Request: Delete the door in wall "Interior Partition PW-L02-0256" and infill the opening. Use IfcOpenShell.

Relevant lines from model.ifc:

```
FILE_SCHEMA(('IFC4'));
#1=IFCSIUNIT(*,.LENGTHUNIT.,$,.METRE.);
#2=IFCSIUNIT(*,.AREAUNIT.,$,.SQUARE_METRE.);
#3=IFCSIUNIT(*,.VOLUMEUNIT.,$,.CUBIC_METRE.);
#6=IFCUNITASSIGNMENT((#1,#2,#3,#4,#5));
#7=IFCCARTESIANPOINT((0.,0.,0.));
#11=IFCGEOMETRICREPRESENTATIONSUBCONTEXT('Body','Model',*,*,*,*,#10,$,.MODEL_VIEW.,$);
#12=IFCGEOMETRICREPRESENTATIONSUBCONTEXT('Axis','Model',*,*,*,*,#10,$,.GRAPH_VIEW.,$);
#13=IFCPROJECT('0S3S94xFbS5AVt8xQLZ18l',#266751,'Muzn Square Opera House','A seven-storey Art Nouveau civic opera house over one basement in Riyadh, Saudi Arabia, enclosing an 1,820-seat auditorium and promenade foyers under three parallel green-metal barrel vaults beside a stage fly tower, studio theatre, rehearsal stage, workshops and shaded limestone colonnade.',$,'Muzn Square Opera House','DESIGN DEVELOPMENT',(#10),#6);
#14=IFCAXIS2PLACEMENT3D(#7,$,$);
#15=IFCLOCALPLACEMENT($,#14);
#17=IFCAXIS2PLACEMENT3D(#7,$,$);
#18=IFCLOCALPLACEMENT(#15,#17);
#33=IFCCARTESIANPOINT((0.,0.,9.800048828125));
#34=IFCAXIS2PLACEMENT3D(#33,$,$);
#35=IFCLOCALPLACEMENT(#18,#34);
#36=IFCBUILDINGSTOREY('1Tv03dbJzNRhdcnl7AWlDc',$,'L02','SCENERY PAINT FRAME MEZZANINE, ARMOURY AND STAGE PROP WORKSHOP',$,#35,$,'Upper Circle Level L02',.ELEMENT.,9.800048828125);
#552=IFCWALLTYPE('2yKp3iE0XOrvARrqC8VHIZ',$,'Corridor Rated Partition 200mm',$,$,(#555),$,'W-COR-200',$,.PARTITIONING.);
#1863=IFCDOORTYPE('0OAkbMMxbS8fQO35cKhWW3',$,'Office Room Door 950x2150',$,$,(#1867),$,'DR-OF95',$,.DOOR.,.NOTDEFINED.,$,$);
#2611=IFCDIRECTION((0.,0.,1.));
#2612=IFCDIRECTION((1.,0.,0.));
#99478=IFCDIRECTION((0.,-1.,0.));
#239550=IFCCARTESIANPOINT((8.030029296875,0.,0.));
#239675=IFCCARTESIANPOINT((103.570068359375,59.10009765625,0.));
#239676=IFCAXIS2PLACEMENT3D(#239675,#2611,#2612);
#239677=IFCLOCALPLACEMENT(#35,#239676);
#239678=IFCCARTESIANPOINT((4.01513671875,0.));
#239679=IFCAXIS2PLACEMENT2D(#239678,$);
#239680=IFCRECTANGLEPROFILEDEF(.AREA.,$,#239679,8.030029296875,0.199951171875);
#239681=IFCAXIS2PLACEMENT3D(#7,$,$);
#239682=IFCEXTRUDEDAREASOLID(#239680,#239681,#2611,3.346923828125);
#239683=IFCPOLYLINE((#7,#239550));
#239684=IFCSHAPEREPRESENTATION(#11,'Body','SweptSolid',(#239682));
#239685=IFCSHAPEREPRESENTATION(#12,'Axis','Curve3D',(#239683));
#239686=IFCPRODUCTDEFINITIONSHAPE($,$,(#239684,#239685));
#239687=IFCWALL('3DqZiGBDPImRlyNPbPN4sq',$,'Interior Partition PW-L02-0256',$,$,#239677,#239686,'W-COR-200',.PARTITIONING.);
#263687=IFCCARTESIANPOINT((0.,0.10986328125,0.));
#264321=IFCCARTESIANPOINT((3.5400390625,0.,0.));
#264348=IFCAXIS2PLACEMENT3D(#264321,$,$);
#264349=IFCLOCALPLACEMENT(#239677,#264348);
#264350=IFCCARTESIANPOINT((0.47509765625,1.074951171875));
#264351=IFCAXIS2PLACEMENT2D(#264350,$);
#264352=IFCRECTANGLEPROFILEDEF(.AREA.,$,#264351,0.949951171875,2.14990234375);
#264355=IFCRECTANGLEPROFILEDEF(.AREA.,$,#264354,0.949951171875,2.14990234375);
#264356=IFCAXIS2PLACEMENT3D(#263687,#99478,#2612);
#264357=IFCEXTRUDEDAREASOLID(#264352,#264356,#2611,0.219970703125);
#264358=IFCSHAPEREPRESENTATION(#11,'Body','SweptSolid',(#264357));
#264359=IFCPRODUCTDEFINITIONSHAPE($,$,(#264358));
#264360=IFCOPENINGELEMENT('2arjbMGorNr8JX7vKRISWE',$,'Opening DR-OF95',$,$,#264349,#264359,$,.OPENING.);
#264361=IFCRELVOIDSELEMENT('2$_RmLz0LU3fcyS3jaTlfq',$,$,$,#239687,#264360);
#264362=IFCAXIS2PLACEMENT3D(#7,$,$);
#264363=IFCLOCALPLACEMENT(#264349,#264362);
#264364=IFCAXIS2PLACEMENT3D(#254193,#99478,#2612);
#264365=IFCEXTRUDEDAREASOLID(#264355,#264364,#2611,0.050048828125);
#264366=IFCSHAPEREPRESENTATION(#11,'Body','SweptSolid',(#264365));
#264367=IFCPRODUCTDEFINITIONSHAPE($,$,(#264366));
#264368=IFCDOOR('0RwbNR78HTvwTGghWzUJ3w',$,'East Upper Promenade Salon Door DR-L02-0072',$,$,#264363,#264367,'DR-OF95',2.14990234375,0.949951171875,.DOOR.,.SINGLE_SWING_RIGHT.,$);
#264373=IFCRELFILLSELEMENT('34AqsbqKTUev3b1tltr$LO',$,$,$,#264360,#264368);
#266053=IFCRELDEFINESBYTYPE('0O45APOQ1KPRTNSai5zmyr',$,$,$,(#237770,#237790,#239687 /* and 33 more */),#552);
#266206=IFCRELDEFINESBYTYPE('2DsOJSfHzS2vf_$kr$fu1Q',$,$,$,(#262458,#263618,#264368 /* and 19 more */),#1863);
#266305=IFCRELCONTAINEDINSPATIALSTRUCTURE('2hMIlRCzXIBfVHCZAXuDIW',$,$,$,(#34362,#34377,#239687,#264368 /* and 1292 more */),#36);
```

```python
import ifcopenshell
import ifcopenshell.api.feature
import ifcopenshell.api.root
import ifcopenshell.geom
import ifcopenshell.util.shape

model = ifcopenshell.open("model.ifc")
settings = ifcopenshell.geom.settings()


def volume(element):
    """Net volume in cubic metres, openings subtracted."""
    shape = ifcopenshell.geom.create_shape(settings, element)
    return ifcopenshell.util.shape.get_volume(shape.geometry)


door = model.by_id(264368)
opening = door.FillsVoids[0].RelatingOpeningElement
wall = opening.VoidsElements[0].RelatingBuildingElement
before = volume(wall)

ifcopenshell.api.root.remove_product(model, product=door)
ifcopenshell.api.feature.remove_feature(model, feature=opening)

after = volume(wall)

print(f"wall volume {before:.3f} -> {after:.3f} m3")

model.write("model-out.ifc")
```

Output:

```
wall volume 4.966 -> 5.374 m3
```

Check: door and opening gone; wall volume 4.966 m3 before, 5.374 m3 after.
